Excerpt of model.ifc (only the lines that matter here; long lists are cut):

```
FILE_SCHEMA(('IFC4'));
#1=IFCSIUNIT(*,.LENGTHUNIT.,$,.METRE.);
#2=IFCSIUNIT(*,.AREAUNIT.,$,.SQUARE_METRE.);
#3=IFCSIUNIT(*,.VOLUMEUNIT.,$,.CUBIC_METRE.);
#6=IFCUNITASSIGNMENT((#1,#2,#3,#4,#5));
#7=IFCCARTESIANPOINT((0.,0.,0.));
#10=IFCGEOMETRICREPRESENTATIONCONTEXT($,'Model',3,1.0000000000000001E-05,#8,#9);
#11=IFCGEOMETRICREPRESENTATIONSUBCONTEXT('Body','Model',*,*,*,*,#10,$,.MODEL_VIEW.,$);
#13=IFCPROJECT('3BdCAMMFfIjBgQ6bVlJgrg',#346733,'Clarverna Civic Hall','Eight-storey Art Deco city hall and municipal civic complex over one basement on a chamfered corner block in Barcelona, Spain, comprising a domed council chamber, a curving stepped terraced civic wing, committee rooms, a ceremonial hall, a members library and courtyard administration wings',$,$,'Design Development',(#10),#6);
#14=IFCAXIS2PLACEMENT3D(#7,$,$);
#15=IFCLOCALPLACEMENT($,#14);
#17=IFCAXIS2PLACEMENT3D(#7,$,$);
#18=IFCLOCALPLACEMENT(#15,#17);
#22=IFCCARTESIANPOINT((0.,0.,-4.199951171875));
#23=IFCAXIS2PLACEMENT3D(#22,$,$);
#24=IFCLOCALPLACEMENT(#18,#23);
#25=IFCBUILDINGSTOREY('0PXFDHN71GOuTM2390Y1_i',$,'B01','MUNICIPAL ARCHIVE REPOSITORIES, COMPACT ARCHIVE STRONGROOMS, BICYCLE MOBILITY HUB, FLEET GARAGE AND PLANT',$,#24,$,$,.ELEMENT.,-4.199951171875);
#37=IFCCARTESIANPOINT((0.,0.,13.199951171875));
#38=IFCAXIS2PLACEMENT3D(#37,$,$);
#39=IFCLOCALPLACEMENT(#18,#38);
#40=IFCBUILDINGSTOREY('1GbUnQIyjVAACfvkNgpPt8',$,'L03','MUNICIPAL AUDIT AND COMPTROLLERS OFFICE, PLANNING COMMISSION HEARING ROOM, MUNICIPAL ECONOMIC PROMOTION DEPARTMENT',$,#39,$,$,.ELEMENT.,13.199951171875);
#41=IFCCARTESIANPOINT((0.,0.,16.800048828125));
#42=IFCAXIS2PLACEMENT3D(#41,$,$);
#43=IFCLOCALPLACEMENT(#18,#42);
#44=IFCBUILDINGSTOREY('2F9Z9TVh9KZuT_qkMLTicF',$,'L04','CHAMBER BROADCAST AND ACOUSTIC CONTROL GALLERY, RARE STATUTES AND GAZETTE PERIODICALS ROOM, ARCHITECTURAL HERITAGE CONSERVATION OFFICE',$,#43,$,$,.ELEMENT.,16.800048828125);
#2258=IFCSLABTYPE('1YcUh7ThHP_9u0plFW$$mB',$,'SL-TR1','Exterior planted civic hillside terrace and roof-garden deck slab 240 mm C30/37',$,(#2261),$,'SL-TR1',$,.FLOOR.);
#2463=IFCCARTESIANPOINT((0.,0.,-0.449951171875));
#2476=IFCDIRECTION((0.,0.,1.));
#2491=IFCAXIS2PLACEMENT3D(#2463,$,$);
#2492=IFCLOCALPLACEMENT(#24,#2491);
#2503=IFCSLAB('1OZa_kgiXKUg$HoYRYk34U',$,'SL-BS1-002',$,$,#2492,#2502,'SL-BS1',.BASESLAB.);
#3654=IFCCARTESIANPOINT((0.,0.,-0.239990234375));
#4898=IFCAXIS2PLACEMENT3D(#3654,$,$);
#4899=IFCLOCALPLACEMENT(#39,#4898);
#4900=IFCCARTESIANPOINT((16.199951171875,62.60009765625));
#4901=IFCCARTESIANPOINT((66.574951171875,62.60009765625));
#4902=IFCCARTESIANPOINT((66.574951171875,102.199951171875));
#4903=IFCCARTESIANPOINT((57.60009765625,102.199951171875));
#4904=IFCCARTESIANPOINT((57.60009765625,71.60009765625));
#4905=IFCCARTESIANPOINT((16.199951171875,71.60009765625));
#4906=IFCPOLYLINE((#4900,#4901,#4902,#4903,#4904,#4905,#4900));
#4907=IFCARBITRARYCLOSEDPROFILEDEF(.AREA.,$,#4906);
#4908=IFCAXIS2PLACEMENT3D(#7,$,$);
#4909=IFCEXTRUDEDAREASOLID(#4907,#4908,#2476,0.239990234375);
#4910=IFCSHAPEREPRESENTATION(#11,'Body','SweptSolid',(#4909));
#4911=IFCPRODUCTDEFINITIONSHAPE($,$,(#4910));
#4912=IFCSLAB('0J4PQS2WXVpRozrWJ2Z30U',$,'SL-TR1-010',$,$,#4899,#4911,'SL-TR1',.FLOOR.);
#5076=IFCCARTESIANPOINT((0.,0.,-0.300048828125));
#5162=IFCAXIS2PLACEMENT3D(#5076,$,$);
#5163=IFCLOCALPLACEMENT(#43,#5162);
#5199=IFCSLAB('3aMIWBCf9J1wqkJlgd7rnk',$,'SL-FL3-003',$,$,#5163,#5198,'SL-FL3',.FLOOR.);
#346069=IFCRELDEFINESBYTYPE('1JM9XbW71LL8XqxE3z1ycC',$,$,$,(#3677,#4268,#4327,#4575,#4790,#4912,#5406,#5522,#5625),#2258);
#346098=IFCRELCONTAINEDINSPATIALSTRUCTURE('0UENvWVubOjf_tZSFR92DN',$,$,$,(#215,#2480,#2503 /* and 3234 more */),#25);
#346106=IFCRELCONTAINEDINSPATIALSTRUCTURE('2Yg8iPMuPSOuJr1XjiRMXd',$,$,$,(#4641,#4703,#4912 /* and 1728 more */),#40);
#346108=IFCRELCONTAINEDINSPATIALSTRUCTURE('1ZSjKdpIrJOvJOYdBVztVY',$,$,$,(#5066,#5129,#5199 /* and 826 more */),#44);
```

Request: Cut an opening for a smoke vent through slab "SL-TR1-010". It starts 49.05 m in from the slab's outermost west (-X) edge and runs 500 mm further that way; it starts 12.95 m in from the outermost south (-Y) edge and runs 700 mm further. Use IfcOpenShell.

```python
import numpy as np
import ifcopenshell
import ifcopenshell.api.feature
import ifcopenshell.api.geometry
import ifcopenshell.api.root
import ifcopenshell.geom
import ifcopenshell.util.placement
import ifcopenshell.util.representation
import ifcopenshell.util.shape
import ifcopenshell.util.unit

model = ifcopenshell.open("model.ifc")
unit_scale = ifcopenshell.util.unit.calculate_unit_scale(model)
settings = ifcopenshell.geom.settings()


def volume(element):
    """Net volume in cubic metres, openings subtracted."""
    shape = ifcopenshell.geom.create_shape(settings, element)
    return ifcopenshell.util.shape.get_volume(shape.geometry)


slab = model.by_id(4912)
before = volume(slab)

# Extent in the slab's own axes, in metres. The edges named are its -X and -Y sides.
slab_shape = ifcopenshell.geom.create_shape(settings, slab)
vertices = ifcopenshell.util.shape.get_vertices(slab_shape.geometry)
x_min, y_min, bottom = vertices.min(axis=0)
top = vertices[:, 2].max()

opening = ifcopenshell.api.root.create_entity(model, ifc_class="IfcOpeningElement", name="Smoke vent opening", predefined_type="OPENING")
context = ifcopenshell.util.representation.get_context(model, "Model", "Body", "MODEL_VIEW")
width, depth = 0.5, 0.7
outline = [(0.0, 0.0), (width, 0.0), (width, depth), (0.0, depth), (0.0, 0.0)]
# Overshoot both faces by 50 mm so the cut is clean.
shape = ifcopenshell.api.geometry.add_slab_representation(
    model, context=context, depth=top - bottom + 0.1, polyline=outline
)
ifcopenshell.api.geometry.assign_representation(model, product=opening, representation=shape)

matrix = ifcopenshell.util.placement.get_local_placement(slab.ObjectPlacement)
matrix[:, 3] = matrix @ np.append(np.array([x_min + 49.05, y_min + 12.95, bottom - 0.05]) / unit_scale, 1.0)
ifcopenshell.api.geometry.edit_object_placement(model, product=opening, matrix=matrix, is_si=False)
ifcopenshell.api.feature.add_feature(model, feature=opening, element=slab)

after = volume(slab)

print(f"slab volume {before:.3f} -> {after:.3f} m3")

model.write("model_edited.ifc")
```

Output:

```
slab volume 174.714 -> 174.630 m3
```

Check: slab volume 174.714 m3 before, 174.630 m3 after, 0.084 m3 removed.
